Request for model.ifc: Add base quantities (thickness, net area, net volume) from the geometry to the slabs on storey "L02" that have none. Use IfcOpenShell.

First a look at what the model holds.

```python
import ifcopenshell
import ifcopenshell.util.element
import ifcopenshell.util.unit

model = ifcopenshell.open("model.ifc")
print(model.schema)
for unit_type in ("LENGTHUNIT", "AREAUNIT", "VOLUMEUNIT"):
    print(unit_type, ifcopenshell.util.unit.calculate_unit_scale(model, unit_type))
storey = next(s for s in model.by_type("IfcBuildingStorey") if s.Name == "L02")
slabs = [e for e in ifcopenshell.util.element.get_decomposition(storey) if e.is_a("IfcSlab")]
for e in sorted(slabs, key=lambda e: e.id()):
    print(e.id(), e.is_a(), e.Name, list(ifcopenshell.util.element.get_psets(e, qtos_only=True)), sep=" | ")
```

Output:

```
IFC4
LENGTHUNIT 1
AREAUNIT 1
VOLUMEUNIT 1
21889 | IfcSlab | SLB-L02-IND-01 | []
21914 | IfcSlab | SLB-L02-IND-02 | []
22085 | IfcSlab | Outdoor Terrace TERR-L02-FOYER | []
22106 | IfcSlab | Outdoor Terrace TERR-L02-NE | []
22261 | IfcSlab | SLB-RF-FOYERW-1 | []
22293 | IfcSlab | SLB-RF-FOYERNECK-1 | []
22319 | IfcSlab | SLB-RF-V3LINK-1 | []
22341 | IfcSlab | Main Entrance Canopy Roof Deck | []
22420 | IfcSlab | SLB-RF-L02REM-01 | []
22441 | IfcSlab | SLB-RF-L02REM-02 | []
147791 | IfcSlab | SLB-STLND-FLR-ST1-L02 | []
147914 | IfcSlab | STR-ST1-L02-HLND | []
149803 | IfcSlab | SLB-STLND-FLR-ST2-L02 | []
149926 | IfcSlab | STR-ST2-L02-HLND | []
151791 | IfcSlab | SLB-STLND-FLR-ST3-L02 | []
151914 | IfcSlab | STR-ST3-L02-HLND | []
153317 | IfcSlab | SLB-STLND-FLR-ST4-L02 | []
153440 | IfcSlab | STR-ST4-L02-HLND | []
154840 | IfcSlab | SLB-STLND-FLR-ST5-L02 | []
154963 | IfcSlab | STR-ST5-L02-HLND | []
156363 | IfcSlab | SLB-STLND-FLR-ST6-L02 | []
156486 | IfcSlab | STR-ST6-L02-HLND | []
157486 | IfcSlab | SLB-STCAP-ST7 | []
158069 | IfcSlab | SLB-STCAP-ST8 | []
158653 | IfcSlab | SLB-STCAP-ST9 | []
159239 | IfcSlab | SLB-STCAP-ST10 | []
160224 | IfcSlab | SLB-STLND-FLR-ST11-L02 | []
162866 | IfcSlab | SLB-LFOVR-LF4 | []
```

```python
import ifcopenshell
import ifcopenshell.api.pset
import ifcopenshell.geom
import ifcopenshell.util.element
import ifcopenshell.util.shape
import ifcopenshell.util.unit

model = ifcopenshell.open("model.ifc")
unit_scale = ifcopenshell.util.unit.calculate_unit_scale(model)
area_scale = ifcopenshell.util.unit.calculate_unit_scale(model, "AREAUNIT")
volume_scale = ifcopenshell.util.unit.calculate_unit_scale(model, "VOLUMEUNIT")
settings = ifcopenshell.geom.settings()

storey = next(s for s in model.by_type("IfcBuildingStorey") if s.Name == "L02")
slabs = [e for e in ifcopenshell.util.element.get_decomposition(storey) if e.is_a("IfcSlab")]

for e in sorted(slabs, key=lambda e: e.id()):
    if ifcopenshell.util.element.get_psets(e, qtos_only=True, should_inherit=False):
        continue
    # Geometry comes back in metres, in the element's own axes.
    shape = ifcopenshell.geom.create_shape(settings, e)
    values = {
        "Width": ifcopenshell.util.shape.get_z(shape.geometry) / unit_scale,
        "NetArea": ifcopenshell.util.shape.get_footprint_area(shape.geometry) / area_scale,
        "NetVolume": ifcopenshell.util.shape.get_volume(shape.geometry) / volume_scale,
    }
    qto = ifcopenshell.api.pset.add_qto(model, product=e, name="Qto_SlabBaseQuantities")
    ifcopenshell.api.pset.edit_qto(model, qto=qto, properties=values)
    print(e.id(), {k: round(v, 3) for k, v in values.items()})

model.write("model-out.ifc")
```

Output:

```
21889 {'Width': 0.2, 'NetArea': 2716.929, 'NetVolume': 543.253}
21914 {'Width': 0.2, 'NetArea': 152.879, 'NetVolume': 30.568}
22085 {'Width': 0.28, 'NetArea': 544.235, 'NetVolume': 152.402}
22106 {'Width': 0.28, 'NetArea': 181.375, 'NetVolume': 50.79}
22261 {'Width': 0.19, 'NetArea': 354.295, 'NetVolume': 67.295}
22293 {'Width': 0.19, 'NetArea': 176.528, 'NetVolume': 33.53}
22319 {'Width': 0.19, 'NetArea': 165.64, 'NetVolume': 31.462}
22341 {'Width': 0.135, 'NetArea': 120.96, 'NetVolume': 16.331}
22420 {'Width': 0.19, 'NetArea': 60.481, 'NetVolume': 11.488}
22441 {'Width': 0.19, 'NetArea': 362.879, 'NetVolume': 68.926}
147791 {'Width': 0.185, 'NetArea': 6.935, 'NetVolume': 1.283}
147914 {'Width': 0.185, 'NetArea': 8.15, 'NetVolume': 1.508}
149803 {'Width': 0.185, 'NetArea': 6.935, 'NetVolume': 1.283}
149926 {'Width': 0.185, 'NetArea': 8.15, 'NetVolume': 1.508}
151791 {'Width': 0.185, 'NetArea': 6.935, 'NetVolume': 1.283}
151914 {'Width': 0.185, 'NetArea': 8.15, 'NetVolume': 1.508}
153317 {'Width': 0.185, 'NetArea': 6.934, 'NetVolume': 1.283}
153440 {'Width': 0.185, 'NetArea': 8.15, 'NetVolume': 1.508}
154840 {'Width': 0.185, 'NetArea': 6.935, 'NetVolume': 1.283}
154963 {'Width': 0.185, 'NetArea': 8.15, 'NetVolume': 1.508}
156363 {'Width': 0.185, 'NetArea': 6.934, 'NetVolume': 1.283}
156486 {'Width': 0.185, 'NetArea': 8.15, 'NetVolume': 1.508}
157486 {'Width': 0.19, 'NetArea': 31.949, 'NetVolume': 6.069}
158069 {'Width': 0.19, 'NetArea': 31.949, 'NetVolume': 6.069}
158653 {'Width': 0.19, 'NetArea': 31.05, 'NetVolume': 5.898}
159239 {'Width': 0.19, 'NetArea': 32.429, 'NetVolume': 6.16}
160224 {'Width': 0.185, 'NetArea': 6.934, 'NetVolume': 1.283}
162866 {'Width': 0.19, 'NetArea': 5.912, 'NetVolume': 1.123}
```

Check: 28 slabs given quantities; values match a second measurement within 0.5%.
